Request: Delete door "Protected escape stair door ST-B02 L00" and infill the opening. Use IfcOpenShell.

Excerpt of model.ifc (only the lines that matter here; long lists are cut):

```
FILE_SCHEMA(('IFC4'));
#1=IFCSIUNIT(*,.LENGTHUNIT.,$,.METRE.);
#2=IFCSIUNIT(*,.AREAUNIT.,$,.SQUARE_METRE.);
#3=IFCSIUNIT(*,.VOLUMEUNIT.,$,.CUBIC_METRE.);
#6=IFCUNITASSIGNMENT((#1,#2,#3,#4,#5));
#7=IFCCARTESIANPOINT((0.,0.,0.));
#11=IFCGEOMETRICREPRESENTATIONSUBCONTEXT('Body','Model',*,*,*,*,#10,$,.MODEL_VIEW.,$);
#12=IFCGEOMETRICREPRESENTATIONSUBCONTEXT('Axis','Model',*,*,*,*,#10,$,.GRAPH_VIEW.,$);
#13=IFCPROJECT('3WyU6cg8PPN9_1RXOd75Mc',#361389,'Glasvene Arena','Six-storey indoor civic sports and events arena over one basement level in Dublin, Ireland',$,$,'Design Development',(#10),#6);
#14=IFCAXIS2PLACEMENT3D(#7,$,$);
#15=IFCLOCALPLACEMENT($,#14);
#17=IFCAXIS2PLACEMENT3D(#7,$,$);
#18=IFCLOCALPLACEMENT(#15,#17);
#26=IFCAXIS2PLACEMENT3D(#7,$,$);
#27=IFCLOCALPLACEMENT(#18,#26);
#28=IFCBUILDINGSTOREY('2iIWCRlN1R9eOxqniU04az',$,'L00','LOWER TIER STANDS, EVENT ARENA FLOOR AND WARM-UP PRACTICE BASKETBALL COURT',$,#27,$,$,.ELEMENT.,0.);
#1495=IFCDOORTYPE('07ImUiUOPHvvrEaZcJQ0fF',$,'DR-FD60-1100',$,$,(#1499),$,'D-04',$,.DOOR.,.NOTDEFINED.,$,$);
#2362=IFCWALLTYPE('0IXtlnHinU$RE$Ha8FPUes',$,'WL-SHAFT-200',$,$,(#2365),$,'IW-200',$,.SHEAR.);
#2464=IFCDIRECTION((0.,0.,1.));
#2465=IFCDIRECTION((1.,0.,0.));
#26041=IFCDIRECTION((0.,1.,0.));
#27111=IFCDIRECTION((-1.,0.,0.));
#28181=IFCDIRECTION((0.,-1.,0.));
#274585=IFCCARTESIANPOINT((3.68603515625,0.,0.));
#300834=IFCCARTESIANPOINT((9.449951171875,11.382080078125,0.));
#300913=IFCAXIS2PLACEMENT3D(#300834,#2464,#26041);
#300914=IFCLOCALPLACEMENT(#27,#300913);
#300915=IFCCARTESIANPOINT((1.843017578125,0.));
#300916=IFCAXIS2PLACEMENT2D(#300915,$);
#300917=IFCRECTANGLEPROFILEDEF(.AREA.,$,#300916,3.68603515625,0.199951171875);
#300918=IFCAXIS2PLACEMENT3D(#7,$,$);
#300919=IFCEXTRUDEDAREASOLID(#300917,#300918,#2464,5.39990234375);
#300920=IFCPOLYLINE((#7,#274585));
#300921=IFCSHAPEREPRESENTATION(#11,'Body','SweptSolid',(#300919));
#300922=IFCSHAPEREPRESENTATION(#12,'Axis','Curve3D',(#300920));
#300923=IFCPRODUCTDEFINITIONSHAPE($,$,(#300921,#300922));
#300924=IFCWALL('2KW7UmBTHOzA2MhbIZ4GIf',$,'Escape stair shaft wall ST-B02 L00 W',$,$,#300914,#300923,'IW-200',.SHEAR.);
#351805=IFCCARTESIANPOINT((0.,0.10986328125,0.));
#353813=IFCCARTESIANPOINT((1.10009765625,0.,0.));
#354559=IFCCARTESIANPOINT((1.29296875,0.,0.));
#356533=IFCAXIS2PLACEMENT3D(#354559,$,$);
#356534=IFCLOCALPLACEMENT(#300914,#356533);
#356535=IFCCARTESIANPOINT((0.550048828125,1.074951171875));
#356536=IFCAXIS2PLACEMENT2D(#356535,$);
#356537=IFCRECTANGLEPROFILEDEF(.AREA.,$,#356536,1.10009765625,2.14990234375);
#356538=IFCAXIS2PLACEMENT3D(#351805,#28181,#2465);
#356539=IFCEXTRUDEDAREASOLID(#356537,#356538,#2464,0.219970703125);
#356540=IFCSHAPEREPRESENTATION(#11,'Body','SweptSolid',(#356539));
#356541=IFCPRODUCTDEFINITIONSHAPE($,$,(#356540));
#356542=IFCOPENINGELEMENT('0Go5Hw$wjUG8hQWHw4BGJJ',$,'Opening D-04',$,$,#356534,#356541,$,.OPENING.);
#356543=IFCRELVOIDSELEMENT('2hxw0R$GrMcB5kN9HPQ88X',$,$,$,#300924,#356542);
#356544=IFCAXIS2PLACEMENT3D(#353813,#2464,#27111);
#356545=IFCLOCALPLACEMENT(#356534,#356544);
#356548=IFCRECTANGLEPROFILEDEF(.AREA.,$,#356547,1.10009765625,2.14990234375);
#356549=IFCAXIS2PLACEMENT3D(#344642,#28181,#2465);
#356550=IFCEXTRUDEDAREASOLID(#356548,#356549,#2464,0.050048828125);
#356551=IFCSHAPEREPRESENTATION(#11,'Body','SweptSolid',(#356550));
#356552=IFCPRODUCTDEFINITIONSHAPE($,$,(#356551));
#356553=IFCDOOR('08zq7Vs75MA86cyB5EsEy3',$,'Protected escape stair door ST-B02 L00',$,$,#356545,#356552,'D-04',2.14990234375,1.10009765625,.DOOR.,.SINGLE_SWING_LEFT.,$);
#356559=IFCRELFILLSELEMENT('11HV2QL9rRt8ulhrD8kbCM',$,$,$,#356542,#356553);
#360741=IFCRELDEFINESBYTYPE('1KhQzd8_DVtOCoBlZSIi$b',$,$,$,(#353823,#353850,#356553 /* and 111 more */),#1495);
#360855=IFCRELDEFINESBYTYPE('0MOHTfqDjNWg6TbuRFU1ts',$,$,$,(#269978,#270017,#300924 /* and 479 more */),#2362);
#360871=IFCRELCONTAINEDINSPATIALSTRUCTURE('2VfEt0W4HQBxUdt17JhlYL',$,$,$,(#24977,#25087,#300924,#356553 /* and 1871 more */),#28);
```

```python
import ifcopenshell
import ifcopenshell.api.feature
import ifcopenshell.api.root
import ifcopenshell.geom
import ifcopenshell.util.shape

model = ifcopenshell.open("model.ifc")
settings = ifcopenshell.geom.settings()


def volume(element):
    """Net volume in cubic metres, openings subtracted."""
    shape = ifcopenshell.geom.create_shape(settings, element)
    return ifcopenshell.util.shape.get_volume(shape.geometry)


door = model.by_guid("08zq7Vs75MA86cyB5EsEy3")
opening = door.FillsVoids[0].RelatingOpeningElement
wall = opening.VoidsElements[0].RelatingBuildingElement
before = volume(wall)

ifcopenshell.api.root.remove_product(model, product=door)
ifcopenshell.api.feature.remove_feature(model, feature=opening)

after = volume(wall)

print(f"wall volume {before:.3f} -> {after:.3f} m3")

model.write("model_v2.ifc")
```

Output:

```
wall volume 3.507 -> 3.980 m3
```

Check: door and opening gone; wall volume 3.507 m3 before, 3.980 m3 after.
